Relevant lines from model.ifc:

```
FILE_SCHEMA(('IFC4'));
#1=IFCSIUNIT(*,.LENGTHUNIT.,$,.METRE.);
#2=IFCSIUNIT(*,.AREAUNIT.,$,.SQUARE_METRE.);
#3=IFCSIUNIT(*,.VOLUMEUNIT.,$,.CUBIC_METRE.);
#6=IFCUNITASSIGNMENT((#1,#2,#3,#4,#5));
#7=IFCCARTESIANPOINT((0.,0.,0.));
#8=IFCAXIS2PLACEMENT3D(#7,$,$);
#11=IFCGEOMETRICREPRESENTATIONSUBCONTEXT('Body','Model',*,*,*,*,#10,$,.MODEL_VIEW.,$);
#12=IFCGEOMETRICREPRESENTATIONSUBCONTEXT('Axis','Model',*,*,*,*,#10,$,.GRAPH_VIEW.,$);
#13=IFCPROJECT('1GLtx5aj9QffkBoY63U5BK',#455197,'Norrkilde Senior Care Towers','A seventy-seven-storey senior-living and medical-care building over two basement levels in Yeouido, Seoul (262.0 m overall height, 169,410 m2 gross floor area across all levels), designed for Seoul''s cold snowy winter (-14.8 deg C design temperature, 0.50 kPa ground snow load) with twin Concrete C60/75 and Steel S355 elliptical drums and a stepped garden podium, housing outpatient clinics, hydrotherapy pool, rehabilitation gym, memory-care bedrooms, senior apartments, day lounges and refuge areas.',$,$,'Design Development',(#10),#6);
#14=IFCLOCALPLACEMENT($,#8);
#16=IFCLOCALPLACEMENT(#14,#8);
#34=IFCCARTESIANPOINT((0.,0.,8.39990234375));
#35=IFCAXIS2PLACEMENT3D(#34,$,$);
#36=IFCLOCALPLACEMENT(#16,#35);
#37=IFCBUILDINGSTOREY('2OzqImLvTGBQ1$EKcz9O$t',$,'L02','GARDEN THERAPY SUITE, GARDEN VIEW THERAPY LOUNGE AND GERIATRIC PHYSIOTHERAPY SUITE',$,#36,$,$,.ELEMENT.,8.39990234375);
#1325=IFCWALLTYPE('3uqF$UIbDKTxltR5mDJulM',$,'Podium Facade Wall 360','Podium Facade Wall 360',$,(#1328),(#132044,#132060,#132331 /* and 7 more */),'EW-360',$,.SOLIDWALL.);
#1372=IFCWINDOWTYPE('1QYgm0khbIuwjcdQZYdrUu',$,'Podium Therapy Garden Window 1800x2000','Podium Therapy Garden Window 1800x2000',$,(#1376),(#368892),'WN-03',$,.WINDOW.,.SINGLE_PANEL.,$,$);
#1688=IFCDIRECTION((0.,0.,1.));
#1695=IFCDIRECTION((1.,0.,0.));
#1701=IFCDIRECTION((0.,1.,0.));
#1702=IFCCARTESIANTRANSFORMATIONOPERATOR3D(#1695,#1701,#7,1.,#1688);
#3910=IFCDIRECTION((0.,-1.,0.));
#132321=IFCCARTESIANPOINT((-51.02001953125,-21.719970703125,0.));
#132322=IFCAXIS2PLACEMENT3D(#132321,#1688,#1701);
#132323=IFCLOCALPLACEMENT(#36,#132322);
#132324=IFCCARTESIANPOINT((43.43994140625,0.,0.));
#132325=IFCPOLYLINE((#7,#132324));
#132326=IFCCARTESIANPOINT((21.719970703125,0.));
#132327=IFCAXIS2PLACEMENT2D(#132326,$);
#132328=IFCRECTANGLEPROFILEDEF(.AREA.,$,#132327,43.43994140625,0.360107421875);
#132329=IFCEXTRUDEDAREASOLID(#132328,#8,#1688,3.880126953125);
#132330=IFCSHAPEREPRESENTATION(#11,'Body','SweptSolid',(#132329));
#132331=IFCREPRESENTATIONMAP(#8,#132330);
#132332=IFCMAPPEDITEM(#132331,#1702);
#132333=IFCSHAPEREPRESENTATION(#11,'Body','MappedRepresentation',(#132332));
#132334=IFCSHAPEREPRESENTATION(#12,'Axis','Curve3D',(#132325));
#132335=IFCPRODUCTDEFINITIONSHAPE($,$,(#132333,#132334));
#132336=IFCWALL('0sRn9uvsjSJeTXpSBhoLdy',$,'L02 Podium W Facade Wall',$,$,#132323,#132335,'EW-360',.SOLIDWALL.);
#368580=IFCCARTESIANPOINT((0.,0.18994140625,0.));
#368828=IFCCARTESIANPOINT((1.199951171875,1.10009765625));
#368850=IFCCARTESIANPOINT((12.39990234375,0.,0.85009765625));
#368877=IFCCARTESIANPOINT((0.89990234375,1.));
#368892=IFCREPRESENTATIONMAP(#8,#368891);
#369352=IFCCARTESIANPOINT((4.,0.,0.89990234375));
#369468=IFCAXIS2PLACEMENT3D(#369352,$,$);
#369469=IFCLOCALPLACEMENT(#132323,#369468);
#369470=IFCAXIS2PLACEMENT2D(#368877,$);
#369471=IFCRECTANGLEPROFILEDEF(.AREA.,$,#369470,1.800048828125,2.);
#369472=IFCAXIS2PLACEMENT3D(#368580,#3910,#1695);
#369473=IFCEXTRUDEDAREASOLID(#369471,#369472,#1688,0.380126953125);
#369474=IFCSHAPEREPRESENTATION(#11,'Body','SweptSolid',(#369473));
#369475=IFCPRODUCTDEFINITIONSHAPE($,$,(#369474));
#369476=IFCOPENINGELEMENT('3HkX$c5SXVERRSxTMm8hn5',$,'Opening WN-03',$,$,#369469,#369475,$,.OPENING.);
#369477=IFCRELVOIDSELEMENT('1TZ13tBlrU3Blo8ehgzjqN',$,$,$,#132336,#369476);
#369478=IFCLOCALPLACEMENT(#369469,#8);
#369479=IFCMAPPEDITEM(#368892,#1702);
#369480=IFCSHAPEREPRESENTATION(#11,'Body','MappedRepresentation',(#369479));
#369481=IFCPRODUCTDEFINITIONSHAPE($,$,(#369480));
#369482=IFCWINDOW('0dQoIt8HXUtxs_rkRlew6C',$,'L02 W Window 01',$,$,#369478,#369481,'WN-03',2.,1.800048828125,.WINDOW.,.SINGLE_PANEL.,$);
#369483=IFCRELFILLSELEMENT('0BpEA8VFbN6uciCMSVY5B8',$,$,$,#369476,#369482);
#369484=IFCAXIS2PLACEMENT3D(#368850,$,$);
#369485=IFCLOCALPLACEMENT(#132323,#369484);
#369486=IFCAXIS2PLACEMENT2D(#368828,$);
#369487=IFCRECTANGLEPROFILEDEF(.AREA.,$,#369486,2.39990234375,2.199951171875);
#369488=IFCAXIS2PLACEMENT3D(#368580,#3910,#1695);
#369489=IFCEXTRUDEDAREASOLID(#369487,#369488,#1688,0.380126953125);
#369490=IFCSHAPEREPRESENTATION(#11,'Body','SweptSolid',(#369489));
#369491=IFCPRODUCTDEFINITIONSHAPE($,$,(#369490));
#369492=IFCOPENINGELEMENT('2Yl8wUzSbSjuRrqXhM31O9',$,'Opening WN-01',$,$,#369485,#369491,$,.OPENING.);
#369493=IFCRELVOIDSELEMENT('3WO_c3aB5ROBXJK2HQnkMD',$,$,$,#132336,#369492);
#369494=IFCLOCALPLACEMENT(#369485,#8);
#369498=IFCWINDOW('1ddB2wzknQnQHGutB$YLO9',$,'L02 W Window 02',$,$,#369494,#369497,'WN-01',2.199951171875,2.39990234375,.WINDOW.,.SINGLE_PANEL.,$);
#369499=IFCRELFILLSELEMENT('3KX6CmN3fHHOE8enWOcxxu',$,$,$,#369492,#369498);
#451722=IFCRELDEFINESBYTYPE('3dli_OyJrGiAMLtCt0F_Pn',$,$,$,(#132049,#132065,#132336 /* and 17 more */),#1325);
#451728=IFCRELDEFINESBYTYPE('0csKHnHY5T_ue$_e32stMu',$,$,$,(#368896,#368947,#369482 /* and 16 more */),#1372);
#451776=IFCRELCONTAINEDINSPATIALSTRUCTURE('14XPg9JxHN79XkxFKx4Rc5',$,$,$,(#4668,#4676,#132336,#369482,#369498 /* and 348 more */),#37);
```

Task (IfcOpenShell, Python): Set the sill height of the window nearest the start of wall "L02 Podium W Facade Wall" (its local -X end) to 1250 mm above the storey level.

```python
import numpy as np
import ifcopenshell
import ifcopenshell.api.geometry
import ifcopenshell.geom
import ifcopenshell.util.element
import ifcopenshell.util.placement
import ifcopenshell.util.shape
import ifcopenshell.util.unit

model = ifcopenshell.open("model.ifc")
unit_scale = ifcopenshell.util.unit.calculate_unit_scale(model)

window = model.by_guid("0dQoIt8HXUtxs_rkRlew6C")
opening = window.FillsVoids[0].RelatingOpeningElement
storey = ifcopenshell.util.element.get_container(window, ifc_class="IfcBuildingStorey")
level = ifcopenshell.util.placement.get_local_placement(storey.ObjectPlacement)[2, 3]

# The opening's origin need not be at the sill, so measure its lowest point.
shape = ifcopenshell.geom.create_shape(ifcopenshell.geom.settings(), opening)
bottom = ifcopenshell.util.shape.get_shape_bottom_elevation(shape, shape.geometry) / unit_scale
dz = level + 1.25 / unit_scale - bottom

shift = np.array([0.0, 0.0, dz])
# The window is placed relative to its opening, so it follows when the opening moves.
matrix = ifcopenshell.util.placement.get_local_placement(opening.ObjectPlacement)
matrix[:3, 3] += shift
ifcopenshell.api.geometry.edit_object_placement(
    model, product=opening, matrix=matrix, is_si=False, should_transform_children=True
)

print(f"moved by {dz * unit_scale:+.3f} m")

model.write("model_updated.ifc")
```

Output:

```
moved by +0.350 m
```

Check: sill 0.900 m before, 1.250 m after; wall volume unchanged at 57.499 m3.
